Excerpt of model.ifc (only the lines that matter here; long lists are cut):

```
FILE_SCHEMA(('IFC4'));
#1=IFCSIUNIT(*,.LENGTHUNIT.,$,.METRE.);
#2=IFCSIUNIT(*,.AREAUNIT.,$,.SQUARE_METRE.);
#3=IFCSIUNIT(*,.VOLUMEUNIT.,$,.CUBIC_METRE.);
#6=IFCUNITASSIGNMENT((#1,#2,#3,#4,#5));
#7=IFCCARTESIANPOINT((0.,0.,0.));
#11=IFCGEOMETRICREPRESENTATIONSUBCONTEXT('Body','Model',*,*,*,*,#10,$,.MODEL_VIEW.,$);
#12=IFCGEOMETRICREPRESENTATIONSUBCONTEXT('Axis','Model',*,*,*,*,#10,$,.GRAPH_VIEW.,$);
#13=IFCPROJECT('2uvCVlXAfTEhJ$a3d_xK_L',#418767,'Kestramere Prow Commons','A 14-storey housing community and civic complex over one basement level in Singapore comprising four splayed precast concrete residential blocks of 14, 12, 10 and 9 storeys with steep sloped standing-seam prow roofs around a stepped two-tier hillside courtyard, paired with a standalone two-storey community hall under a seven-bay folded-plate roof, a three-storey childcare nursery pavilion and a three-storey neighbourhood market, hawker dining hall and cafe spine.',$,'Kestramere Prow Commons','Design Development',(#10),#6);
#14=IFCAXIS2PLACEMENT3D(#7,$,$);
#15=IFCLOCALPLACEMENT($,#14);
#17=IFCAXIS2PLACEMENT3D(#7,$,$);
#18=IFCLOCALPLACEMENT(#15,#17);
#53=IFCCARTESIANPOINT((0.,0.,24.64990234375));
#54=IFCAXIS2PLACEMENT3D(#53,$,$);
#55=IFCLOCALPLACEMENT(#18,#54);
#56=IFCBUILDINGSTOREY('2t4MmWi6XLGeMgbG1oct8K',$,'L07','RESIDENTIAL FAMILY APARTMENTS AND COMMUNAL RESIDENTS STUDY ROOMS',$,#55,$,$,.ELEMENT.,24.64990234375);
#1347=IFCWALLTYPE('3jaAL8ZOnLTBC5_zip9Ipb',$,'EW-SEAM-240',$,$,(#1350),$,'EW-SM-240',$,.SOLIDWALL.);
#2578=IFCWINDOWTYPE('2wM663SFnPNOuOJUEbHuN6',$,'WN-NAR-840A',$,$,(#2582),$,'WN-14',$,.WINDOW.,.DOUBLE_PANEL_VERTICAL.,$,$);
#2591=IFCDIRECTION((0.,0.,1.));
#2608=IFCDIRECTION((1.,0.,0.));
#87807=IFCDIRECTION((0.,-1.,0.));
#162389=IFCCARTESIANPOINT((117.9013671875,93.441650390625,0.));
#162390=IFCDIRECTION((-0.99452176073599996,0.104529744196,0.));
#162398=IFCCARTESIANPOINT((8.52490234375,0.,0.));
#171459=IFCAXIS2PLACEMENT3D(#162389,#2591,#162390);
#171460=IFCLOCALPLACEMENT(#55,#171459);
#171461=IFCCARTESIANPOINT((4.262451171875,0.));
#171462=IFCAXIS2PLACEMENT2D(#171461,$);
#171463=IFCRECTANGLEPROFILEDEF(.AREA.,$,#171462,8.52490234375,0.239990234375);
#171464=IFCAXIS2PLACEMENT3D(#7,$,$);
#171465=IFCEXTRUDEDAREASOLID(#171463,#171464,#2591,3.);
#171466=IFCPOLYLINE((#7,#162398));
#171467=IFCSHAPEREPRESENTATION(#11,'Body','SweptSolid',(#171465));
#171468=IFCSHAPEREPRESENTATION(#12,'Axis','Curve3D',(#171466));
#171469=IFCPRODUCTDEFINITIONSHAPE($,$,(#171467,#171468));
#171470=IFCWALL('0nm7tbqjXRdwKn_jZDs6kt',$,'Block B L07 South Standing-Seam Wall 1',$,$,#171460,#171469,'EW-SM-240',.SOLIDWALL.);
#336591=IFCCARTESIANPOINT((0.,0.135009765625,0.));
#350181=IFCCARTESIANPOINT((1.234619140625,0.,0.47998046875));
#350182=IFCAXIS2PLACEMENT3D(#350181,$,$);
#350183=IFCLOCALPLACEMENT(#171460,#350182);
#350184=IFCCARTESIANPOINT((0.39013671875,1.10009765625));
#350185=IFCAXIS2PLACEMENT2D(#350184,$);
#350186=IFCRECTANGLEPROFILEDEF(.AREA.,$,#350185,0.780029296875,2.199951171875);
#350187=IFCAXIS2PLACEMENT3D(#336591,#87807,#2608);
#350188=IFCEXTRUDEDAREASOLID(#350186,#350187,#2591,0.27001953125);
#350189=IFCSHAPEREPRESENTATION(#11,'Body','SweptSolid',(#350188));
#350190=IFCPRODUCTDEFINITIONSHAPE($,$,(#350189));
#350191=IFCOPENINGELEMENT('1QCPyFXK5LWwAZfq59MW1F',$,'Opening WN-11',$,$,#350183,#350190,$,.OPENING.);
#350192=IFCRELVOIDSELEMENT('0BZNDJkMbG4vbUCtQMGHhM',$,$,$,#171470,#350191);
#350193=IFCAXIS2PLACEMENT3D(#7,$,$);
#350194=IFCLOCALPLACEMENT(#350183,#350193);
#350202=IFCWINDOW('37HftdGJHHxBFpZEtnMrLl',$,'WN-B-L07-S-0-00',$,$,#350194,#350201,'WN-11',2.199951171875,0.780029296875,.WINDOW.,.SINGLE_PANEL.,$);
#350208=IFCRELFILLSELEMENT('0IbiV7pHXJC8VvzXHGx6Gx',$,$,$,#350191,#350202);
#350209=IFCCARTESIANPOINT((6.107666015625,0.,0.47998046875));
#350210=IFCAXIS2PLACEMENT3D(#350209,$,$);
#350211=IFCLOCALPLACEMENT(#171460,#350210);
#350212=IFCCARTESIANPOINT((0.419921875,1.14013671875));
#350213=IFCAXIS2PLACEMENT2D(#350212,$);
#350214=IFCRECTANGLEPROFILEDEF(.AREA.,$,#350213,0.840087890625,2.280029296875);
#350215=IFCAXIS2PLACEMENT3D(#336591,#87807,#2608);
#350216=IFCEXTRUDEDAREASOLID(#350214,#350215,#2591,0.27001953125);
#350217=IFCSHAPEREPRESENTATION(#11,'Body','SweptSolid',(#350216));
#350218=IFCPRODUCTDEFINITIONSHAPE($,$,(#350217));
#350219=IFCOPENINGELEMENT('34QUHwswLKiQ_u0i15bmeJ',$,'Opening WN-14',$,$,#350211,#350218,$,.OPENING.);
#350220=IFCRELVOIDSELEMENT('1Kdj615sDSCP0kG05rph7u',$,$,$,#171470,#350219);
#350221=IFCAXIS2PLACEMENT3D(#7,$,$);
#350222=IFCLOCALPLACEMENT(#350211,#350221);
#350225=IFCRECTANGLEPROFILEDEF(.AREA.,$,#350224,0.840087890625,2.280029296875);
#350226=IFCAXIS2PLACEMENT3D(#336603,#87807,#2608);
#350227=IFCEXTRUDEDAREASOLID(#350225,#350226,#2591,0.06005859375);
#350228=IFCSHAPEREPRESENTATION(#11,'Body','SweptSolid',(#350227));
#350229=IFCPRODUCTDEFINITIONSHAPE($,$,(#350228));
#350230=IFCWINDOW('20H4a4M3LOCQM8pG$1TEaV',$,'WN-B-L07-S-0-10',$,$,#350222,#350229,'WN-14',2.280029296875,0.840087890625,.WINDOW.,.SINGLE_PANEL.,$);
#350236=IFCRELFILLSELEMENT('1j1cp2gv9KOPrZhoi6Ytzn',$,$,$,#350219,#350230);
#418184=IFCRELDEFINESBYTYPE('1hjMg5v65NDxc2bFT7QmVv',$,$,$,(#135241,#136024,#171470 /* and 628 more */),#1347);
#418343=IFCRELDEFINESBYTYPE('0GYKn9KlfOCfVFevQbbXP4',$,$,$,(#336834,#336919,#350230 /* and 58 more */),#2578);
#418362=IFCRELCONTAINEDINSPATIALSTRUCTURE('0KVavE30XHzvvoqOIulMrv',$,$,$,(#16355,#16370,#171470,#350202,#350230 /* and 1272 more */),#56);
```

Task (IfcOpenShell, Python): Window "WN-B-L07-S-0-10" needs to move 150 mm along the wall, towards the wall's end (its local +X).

```python
import ifcopenshell
import ifcopenshell.api.geometry
import ifcopenshell.util.placement
import ifcopenshell.util.unit

model = ifcopenshell.open("model.ifc")
unit_scale = ifcopenshell.util.unit.calculate_unit_scale(model)

window = model.by_guid("20H4a4M3LOCQM8pG$1TEaV")
opening = window.FillsVoids[0].RelatingOpeningElement
wall = opening.VoidsElements[0].RelatingBuildingElement

wall_matrix = ifcopenshell.util.placement.get_local_placement(wall.ObjectPlacement)
shift = wall_matrix[:3, 0] * 0.15 / unit_scale
before = ifcopenshell.util.placement.get_local_placement(window.ObjectPlacement)[:3, 3].copy()

# The window is placed relative to its opening, so it follows when the opening moves.
matrix = ifcopenshell.util.placement.get_local_placement(opening.ObjectPlacement)
matrix[:3, 3] += shift
ifcopenshell.api.geometry.edit_object_placement(
    model, product=opening, matrix=matrix, is_si=False, should_transform_children=True
)

after = ifcopenshell.util.placement.get_local_placement(window.ObjectPlacement)[:3, 3]
print("window moved by", (after - before).round(3) + 0.0)

model.write("model_rev.ifc")
```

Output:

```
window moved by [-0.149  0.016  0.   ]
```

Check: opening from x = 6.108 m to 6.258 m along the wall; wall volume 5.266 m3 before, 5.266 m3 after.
